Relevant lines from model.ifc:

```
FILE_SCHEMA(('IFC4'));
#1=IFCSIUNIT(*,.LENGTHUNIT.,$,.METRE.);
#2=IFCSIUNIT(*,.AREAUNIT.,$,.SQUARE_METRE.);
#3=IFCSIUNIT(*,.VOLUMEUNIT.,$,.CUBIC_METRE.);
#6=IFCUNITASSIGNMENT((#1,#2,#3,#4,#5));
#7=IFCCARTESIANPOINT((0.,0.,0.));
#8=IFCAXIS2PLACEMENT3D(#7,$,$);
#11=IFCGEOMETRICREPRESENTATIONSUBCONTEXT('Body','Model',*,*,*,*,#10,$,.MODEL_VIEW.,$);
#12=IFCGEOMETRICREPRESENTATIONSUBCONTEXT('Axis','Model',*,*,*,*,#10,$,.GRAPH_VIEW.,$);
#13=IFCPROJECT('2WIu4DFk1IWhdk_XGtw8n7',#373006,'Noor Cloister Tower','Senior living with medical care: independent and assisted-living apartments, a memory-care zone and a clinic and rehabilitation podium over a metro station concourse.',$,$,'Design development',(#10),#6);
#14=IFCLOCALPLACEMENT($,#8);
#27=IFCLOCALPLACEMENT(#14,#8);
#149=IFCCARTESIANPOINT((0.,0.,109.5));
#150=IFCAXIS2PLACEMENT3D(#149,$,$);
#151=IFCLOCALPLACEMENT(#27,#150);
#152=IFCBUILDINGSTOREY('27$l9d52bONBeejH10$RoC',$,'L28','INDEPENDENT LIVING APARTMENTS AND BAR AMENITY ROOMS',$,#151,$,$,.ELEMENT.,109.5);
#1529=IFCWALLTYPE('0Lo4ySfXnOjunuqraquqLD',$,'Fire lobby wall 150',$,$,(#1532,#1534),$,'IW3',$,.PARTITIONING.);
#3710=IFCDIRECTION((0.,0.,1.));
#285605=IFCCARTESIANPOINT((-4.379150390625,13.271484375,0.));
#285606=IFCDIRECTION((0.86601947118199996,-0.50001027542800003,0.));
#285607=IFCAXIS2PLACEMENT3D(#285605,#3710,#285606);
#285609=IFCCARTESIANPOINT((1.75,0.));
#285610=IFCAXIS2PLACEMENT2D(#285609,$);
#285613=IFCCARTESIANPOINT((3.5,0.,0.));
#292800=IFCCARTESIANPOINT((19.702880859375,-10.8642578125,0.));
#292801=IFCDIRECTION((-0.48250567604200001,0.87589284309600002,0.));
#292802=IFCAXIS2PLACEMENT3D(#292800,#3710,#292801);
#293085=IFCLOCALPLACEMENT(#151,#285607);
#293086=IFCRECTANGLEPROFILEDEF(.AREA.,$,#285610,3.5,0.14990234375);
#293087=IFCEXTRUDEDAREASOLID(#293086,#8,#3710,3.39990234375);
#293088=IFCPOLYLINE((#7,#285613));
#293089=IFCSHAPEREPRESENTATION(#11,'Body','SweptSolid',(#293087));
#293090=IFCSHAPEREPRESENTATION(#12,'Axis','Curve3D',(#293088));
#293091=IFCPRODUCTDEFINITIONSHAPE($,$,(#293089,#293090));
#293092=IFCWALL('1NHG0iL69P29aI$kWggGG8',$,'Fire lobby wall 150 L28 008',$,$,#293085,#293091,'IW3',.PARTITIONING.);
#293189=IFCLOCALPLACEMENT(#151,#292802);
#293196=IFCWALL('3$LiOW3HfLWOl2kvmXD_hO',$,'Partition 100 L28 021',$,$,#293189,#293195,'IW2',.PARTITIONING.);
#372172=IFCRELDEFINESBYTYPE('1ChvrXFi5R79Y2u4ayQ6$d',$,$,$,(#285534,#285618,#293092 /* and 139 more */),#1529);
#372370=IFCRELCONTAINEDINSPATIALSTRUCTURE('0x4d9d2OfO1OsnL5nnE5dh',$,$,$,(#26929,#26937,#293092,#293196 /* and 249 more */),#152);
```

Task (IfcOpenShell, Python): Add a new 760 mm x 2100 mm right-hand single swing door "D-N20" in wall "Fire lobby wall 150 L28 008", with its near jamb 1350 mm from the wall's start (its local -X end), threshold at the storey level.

```python
import numpy as np
import ifcopenshell
import ifcopenshell.api.feature
import ifcopenshell.api.geometry
import ifcopenshell.api.root
import ifcopenshell.api.spatial
import ifcopenshell.geom
import ifcopenshell.util.element
import ifcopenshell.util.placement
import ifcopenshell.util.representation
import ifcopenshell.util.shape
import ifcopenshell.util.unit

model = ifcopenshell.open("model.ifc")
unit_scale = ifcopenshell.util.unit.calculate_unit_scale(model)
settings = ifcopenshell.geom.settings()


def volume(element):
    """Net volume in cubic metres, openings subtracted."""
    shape = ifcopenshell.geom.create_shape(settings, element)
    return ifcopenshell.util.shape.get_volume(shape.geometry)


wall = model.by_guid("1NHG0iL69P29aI$kWggGG8")
storey = ifcopenshell.util.element.get_container(wall, ifc_class="IfcBuildingStorey")
context = ifcopenshell.util.representation.get_context(model, "Model", "Body", "MODEL_VIEW")
before = volume(wall)

width, height, from_end, sill = 0.76, 2.1, 1.35, 0.0  # metres

# The wall runs along its own X axis, and the end named is its -X end.
wall_shape = ifcopenshell.geom.create_shape(settings, wall)
x, y, z = ifcopenshell.util.shape.get_vertices(wall_shape.geometry).T
start = x.min() + from_end
face, thickness = float(y.min()), float(y.max() - y.min())
wall_matrix = ifcopenshell.util.placement.get_local_placement(wall.ObjectPlacement)
level = ifcopenshell.util.placement.get_local_placement(storey.ObjectPlacement)[2, 3]


def in_wall(x, y):
    """Placement at x, y metres in the wall's axes, at sill height."""
    matrix = wall_matrix.copy()
    matrix[:, 3] = wall_matrix @ np.array([x / unit_scale, y / unit_scale, 0.0, 1.0])
    matrix[2, 3] = level + sill / unit_scale
    return matrix


# Opening: a box that overshoots both wall faces by 50 mm.
opening = ifcopenshell.api.root.create_entity(model, ifc_class="IfcOpeningElement", predefined_type="OPENING")
box = ifcopenshell.api.geometry.add_wall_representation(
    model, context=context, length=width, height=height, thickness=thickness + 0.1
)
ifcopenshell.api.geometry.assign_representation(model, product=opening, representation=box)
ifcopenshell.api.geometry.edit_object_placement(model, product=opening, matrix=in_wall(start, face - 0.05), is_si=False)
ifcopenshell.api.feature.add_feature(model, feature=opening, element=wall)

door = ifcopenshell.api.root.create_entity(model, ifc_class="IfcDoor", name="D-N20", predefined_type="DOOR")
door.OverallWidth, door.OverallHeight = width / unit_scale, height / unit_scale
door.OperationType = "SINGLE_SWING_RIGHT"
body = ifcopenshell.api.geometry.add_door_representation(
    model,
    context=context,
    overall_width=door.OverallWidth,
    overall_height=door.OverallHeight,
    operation_type="SINGLE_SWING_RIGHT",
    lining_properties={"LiningDepth": thickness / unit_scale, "ThresholdDepth": thickness / unit_scale},
)
ifcopenshell.api.geometry.assign_representation(model, product=door, representation=body)
ifcopenshell.api.spatial.assign_container(model, products=[door], relating_structure=storey)
ifcopenshell.api.feature.add_filling(model, opening=opening, element=door)

# The lining spans the wall, so the door starts at the wall face.
ifcopenshell.api.geometry.edit_object_placement(model, product=door, matrix=in_wall(start, face), is_si=False)

after = volume(wall)

print(f"wall volume {before:.3f} -> {after:.3f} m3")

model.write("model_rev.ifc")
```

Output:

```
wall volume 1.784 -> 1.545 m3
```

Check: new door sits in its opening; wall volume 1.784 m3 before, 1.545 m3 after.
